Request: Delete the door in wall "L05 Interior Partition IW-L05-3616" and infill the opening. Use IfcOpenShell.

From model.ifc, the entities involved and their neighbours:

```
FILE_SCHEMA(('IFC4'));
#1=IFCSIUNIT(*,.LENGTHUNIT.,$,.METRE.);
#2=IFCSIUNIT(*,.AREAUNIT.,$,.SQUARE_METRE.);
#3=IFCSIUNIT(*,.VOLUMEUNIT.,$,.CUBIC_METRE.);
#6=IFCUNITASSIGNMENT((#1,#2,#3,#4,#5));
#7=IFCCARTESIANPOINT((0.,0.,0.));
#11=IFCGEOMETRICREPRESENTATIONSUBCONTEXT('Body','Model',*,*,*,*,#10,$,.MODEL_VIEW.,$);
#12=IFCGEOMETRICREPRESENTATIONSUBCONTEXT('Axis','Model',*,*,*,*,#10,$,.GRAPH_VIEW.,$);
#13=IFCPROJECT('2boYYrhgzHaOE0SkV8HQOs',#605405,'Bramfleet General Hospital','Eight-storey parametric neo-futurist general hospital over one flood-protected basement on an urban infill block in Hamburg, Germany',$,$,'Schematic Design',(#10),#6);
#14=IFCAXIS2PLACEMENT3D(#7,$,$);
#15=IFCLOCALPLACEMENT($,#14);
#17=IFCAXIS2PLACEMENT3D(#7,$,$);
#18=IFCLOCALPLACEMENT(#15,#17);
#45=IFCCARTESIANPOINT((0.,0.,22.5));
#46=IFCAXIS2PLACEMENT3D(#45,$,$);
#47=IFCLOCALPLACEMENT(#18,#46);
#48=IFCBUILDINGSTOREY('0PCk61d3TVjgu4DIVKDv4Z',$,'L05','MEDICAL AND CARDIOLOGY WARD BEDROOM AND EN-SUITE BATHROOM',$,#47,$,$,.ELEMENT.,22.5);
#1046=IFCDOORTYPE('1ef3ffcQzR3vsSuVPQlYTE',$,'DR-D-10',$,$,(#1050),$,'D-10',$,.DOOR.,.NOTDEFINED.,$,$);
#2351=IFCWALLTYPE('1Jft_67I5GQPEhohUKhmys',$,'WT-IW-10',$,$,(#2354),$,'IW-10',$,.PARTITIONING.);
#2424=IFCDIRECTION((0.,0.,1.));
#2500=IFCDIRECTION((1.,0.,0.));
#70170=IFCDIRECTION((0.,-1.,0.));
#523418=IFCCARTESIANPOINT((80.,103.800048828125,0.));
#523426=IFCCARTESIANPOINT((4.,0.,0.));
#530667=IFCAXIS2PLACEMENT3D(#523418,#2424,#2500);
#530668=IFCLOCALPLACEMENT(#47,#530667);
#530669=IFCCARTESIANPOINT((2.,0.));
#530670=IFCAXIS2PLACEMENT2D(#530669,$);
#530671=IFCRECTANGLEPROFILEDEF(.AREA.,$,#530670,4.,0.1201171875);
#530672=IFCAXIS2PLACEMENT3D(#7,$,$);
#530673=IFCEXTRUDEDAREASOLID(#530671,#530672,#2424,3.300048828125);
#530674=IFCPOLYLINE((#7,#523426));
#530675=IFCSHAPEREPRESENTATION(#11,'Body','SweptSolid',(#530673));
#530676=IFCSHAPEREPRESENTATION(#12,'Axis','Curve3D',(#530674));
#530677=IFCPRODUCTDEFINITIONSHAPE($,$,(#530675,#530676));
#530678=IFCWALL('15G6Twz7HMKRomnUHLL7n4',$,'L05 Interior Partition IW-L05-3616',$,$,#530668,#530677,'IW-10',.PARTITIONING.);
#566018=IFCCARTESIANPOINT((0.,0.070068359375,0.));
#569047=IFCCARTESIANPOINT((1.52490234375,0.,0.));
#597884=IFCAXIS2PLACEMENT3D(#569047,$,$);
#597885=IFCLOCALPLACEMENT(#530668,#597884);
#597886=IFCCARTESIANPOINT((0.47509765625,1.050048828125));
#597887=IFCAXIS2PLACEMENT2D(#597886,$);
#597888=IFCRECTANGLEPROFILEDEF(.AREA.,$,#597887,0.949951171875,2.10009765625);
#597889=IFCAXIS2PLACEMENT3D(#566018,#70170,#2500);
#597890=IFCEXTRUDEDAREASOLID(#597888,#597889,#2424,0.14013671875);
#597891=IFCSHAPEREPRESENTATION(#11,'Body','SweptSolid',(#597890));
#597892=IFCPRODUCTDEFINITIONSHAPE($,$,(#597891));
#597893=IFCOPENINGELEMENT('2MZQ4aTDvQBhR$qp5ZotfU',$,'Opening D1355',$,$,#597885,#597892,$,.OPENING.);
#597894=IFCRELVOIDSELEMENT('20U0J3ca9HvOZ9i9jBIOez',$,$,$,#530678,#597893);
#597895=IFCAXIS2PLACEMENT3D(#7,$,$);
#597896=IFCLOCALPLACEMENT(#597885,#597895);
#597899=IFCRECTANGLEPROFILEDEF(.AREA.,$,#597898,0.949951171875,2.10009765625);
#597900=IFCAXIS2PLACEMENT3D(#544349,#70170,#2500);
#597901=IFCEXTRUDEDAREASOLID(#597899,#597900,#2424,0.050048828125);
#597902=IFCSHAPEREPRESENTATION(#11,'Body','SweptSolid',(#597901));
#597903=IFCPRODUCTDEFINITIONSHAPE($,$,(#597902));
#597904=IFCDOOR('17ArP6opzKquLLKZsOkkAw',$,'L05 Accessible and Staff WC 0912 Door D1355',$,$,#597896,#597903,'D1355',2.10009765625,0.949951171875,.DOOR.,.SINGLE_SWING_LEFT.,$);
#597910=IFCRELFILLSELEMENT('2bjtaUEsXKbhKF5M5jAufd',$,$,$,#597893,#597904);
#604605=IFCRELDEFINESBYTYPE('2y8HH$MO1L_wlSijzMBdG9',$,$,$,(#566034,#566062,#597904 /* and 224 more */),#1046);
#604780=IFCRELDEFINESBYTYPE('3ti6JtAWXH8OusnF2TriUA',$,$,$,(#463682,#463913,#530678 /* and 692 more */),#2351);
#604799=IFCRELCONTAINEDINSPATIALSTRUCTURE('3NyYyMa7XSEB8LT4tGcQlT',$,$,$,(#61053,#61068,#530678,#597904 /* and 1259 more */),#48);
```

```python
import ifcopenshell
import ifcopenshell.api.feature
import ifcopenshell.api.root
import ifcopenshell.geom
import ifcopenshell.util.shape

model = ifcopenshell.open("model.ifc")
settings = ifcopenshell.geom.settings()


def volume(element):
    """Net volume in cubic metres, openings subtracted."""
    shape = ifcopenshell.geom.create_shape(settings, element)
    return ifcopenshell.util.shape.get_volume(shape.geometry)


door = model.by_guid("17ArP6opzKquLLKZsOkkAw")
opening = door.FillsVoids[0].RelatingOpeningElement
wall = opening.VoidsElements[0].RelatingBuildingElement
before = volume(wall)

ifcopenshell.api.root.remove_product(model, product=door)
ifcopenshell.api.feature.remove_feature(model, feature=opening)

after = volume(wall)

print(f"wall volume {before:.3f} -> {after:.3f} m3")

model.write("model_updated.ifc")
```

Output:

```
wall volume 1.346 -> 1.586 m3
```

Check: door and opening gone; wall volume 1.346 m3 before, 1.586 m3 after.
